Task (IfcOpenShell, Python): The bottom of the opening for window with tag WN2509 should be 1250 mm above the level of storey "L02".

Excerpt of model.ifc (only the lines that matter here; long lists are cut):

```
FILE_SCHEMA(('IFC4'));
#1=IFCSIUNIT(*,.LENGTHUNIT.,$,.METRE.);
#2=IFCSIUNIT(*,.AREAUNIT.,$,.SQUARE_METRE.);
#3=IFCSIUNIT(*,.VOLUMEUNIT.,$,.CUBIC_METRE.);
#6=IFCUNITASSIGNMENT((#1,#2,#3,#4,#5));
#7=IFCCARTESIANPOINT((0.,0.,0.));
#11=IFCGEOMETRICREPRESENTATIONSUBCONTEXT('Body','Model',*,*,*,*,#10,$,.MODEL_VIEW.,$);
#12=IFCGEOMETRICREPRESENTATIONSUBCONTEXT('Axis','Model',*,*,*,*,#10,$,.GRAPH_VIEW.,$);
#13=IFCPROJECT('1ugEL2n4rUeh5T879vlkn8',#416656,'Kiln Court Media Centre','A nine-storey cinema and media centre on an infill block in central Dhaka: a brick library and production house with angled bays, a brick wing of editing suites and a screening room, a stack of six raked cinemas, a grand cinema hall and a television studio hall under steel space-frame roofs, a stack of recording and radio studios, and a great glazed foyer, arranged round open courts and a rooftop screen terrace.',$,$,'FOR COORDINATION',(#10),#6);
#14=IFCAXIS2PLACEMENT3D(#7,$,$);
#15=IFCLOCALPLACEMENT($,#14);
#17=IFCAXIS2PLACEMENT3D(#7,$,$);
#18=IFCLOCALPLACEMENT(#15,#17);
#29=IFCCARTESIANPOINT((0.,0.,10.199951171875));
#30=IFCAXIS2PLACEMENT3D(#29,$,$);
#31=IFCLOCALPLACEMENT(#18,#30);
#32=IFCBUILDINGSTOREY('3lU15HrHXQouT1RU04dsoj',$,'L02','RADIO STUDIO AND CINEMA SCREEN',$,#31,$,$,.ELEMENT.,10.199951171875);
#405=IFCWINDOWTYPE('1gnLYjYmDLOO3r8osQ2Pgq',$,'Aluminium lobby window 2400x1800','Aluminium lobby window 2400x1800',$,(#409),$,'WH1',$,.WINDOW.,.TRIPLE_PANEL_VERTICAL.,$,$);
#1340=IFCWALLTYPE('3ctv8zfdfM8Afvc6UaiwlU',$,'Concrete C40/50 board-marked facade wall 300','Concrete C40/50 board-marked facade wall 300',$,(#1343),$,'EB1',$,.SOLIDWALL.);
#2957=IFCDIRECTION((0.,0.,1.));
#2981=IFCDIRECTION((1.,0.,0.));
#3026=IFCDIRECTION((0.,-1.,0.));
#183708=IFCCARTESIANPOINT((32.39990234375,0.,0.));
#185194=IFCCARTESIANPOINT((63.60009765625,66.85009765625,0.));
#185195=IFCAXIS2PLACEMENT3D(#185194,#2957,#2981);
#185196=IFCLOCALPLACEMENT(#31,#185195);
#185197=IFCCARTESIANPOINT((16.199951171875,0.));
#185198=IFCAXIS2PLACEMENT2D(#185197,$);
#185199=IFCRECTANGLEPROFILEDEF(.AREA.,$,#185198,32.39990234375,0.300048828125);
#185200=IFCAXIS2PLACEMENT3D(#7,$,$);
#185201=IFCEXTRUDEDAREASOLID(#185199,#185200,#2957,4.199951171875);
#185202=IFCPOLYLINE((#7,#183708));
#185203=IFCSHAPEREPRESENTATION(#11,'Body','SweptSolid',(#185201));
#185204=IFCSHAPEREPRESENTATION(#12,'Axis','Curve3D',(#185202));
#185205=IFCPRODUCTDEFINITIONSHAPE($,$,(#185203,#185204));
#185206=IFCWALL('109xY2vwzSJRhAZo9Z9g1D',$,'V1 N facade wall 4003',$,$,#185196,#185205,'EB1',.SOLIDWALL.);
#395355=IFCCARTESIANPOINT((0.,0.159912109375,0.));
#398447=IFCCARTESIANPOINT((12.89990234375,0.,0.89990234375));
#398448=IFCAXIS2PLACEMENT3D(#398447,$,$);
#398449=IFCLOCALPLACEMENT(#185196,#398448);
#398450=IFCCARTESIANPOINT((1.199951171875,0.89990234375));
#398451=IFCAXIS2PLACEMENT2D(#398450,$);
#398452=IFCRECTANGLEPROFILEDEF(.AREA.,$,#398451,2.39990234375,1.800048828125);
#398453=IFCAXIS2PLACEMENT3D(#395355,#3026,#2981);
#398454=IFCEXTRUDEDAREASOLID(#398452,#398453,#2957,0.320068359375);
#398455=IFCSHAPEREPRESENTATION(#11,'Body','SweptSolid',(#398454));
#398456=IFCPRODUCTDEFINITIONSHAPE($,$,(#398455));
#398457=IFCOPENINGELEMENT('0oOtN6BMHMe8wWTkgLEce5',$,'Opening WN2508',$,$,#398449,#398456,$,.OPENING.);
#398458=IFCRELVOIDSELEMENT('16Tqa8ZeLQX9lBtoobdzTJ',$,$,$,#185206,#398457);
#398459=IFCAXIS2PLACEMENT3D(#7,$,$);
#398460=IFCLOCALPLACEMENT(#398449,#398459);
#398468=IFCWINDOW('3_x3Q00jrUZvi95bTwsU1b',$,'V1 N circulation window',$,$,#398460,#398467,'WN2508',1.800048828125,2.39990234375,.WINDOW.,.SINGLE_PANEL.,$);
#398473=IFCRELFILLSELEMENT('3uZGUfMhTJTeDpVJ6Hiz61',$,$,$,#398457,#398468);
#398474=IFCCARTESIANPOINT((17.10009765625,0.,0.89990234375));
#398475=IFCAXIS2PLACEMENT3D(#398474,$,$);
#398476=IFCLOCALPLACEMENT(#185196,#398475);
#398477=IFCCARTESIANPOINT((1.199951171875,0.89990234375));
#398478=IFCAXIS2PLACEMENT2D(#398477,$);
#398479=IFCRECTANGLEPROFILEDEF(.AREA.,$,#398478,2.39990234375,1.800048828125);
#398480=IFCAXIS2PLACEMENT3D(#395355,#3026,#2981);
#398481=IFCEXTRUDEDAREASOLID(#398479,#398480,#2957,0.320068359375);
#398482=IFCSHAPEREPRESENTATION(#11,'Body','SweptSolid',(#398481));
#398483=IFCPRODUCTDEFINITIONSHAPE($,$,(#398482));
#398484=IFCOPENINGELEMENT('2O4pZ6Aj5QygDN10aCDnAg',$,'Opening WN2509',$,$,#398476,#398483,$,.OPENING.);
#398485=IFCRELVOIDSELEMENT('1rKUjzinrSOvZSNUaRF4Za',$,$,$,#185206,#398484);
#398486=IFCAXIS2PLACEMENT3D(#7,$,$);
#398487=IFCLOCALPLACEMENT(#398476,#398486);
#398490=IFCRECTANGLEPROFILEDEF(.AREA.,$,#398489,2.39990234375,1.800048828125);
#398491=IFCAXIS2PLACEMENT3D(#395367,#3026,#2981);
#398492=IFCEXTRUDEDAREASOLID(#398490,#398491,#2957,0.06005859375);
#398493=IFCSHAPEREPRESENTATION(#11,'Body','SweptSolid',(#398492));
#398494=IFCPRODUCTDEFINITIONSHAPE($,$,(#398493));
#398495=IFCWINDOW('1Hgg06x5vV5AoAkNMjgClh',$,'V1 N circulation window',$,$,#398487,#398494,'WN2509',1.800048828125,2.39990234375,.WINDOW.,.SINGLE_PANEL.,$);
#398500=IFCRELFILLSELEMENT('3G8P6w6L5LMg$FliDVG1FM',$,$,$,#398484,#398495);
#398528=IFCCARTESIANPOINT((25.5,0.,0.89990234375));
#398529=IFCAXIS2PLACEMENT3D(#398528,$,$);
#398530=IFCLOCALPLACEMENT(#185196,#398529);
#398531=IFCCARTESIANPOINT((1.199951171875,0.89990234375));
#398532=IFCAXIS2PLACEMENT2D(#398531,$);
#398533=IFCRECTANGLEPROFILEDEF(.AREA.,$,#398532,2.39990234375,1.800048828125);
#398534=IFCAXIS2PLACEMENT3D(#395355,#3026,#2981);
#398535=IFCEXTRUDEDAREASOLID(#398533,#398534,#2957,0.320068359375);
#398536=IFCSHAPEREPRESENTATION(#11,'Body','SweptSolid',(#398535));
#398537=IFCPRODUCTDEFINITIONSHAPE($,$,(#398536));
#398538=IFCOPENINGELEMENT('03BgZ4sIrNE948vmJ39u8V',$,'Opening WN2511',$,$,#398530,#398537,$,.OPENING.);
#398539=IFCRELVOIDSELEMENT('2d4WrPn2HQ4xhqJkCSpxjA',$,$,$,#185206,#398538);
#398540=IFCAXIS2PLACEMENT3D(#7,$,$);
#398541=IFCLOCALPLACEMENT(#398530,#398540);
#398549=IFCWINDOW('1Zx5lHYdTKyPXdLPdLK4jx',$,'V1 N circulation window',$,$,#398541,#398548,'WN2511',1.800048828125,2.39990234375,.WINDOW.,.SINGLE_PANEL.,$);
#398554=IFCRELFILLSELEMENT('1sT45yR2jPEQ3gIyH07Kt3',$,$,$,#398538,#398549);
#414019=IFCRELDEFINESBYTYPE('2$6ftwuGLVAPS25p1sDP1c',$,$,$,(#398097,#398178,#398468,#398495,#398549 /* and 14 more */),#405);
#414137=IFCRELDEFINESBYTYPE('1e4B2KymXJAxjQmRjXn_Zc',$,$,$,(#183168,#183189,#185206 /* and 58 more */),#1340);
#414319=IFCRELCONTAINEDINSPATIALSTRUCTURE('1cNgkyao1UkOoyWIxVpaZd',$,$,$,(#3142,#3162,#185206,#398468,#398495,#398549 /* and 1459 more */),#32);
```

```python
import numpy as np
import ifcopenshell
import ifcopenshell.api.geometry
import ifcopenshell.geom
import ifcopenshell.util.element
import ifcopenshell.util.placement
import ifcopenshell.util.shape
import ifcopenshell.util.unit

model = ifcopenshell.open("model.ifc")
unit_scale = ifcopenshell.util.unit.calculate_unit_scale(model)

window = model.by_guid("1Hgg06x5vV5AoAkNMjgClh")
opening = window.FillsVoids[0].RelatingOpeningElement
storey = ifcopenshell.util.element.get_container(window, ifc_class="IfcBuildingStorey")
level = ifcopenshell.util.placement.get_local_placement(storey.ObjectPlacement)[2, 3]

# The opening's origin need not be at the sill, so measure its lowest point.
shape = ifcopenshell.geom.create_shape(ifcopenshell.geom.settings(), opening)
bottom = ifcopenshell.util.shape.get_shape_bottom_elevation(shape, shape.geometry) / unit_scale
dz = level + 1.25 - bottom

shift = np.array([0.0, 0.0, dz])
# The window is placed relative to its opening, so it follows when the opening moves.
matrix = ifcopenshell.util.placement.get_local_placement(opening.ObjectPlacement)
matrix[:3, 3] += shift
ifcopenshell.api.geometry.edit_object_placement(
    model, product=opening, matrix=matrix, is_si=False, should_transform_children=True
)

print(f"moved by {dz * unit_scale:+.3f} m")

model.write("model_updated.ifc")
```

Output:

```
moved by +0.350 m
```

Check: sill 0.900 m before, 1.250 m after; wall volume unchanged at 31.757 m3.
